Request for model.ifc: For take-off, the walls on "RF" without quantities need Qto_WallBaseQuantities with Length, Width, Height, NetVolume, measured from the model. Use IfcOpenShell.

First a look at what the model holds.

```python
import ifcopenshell
import ifcopenshell.util.element
import ifcopenshell.util.unit

model = ifcopenshell.open("model.ifc")
print(model.schema)
for unit_type in ("LENGTHUNIT", "AREAUNIT", "VOLUMEUNIT"):
    print(unit_type, ifcopenshell.util.unit.calculate_unit_scale(model, unit_type))
storey = next(s for s in model.by_type("IfcBuildingStorey") if s.Name == "RF")
walls = [e for e in ifcopenshell.util.element.get_decomposition(storey) if e.is_a("IfcWall")]
for e in sorted(walls, key=lambda e: e.id()):
    print(e.id(), e.is_a(), e.Name, list(ifcopenshell.util.element.get_psets(e, qtos_only=True)), sep=" | ")
```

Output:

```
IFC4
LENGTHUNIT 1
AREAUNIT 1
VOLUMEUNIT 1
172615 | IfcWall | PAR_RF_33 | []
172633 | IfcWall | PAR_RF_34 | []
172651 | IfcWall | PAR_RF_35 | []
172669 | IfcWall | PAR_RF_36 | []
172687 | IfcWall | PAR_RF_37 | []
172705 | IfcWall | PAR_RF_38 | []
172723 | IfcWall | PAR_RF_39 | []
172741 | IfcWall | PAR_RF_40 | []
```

```python
import ifcopenshell
import ifcopenshell.api.pset
import ifcopenshell.geom
import ifcopenshell.util.element
import ifcopenshell.util.shape
import ifcopenshell.util.unit

model = ifcopenshell.open("model.ifc")
unit_scale = ifcopenshell.util.unit.calculate_unit_scale(model)
volume_scale = ifcopenshell.util.unit.calculate_unit_scale(model, "VOLUMEUNIT")
settings = ifcopenshell.geom.settings()

storey = next(s for s in model.by_type("IfcBuildingStorey") if s.Name == "RF")
walls = [e for e in ifcopenshell.util.element.get_decomposition(storey) if e.is_a("IfcWall")]

for e in sorted(walls, key=lambda e: e.id()):
    if ifcopenshell.util.element.get_psets(e, qtos_only=True, should_inherit=False):
        continue
    # Geometry comes back in metres, in the element's own axes.
    shape = ifcopenshell.geom.create_shape(settings, e)
    values = {
        "Length": ifcopenshell.util.shape.get_x(shape.geometry) / unit_scale,
        "Width": ifcopenshell.util.shape.get_y(shape.geometry) / unit_scale,
        "Height": ifcopenshell.util.shape.get_z(shape.geometry) / unit_scale,
        "NetVolume": ifcopenshell.util.shape.get_volume(shape.geometry) / volume_scale,
    }
    qto = ifcopenshell.api.pset.add_qto(model, product=e, name="Qto_WallBaseQuantities")
    ifcopenshell.api.pset.edit_qto(model, qto=qto, properties=values)
    print(e.id(), {k: round(v, 3) for k, v in values.items()})

model.write("model-out.ifc")
```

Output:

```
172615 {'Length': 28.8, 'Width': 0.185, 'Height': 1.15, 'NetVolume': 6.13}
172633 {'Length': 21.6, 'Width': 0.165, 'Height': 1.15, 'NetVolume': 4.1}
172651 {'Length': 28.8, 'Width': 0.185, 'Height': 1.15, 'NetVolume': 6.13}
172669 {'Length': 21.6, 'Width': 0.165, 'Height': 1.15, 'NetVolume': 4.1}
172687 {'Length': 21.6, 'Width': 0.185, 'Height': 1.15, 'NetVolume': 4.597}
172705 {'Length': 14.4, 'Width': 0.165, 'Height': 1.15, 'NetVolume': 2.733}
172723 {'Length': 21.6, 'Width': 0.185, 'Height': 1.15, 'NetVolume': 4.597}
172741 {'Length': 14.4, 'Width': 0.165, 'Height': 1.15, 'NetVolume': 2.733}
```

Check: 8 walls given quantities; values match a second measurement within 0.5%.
